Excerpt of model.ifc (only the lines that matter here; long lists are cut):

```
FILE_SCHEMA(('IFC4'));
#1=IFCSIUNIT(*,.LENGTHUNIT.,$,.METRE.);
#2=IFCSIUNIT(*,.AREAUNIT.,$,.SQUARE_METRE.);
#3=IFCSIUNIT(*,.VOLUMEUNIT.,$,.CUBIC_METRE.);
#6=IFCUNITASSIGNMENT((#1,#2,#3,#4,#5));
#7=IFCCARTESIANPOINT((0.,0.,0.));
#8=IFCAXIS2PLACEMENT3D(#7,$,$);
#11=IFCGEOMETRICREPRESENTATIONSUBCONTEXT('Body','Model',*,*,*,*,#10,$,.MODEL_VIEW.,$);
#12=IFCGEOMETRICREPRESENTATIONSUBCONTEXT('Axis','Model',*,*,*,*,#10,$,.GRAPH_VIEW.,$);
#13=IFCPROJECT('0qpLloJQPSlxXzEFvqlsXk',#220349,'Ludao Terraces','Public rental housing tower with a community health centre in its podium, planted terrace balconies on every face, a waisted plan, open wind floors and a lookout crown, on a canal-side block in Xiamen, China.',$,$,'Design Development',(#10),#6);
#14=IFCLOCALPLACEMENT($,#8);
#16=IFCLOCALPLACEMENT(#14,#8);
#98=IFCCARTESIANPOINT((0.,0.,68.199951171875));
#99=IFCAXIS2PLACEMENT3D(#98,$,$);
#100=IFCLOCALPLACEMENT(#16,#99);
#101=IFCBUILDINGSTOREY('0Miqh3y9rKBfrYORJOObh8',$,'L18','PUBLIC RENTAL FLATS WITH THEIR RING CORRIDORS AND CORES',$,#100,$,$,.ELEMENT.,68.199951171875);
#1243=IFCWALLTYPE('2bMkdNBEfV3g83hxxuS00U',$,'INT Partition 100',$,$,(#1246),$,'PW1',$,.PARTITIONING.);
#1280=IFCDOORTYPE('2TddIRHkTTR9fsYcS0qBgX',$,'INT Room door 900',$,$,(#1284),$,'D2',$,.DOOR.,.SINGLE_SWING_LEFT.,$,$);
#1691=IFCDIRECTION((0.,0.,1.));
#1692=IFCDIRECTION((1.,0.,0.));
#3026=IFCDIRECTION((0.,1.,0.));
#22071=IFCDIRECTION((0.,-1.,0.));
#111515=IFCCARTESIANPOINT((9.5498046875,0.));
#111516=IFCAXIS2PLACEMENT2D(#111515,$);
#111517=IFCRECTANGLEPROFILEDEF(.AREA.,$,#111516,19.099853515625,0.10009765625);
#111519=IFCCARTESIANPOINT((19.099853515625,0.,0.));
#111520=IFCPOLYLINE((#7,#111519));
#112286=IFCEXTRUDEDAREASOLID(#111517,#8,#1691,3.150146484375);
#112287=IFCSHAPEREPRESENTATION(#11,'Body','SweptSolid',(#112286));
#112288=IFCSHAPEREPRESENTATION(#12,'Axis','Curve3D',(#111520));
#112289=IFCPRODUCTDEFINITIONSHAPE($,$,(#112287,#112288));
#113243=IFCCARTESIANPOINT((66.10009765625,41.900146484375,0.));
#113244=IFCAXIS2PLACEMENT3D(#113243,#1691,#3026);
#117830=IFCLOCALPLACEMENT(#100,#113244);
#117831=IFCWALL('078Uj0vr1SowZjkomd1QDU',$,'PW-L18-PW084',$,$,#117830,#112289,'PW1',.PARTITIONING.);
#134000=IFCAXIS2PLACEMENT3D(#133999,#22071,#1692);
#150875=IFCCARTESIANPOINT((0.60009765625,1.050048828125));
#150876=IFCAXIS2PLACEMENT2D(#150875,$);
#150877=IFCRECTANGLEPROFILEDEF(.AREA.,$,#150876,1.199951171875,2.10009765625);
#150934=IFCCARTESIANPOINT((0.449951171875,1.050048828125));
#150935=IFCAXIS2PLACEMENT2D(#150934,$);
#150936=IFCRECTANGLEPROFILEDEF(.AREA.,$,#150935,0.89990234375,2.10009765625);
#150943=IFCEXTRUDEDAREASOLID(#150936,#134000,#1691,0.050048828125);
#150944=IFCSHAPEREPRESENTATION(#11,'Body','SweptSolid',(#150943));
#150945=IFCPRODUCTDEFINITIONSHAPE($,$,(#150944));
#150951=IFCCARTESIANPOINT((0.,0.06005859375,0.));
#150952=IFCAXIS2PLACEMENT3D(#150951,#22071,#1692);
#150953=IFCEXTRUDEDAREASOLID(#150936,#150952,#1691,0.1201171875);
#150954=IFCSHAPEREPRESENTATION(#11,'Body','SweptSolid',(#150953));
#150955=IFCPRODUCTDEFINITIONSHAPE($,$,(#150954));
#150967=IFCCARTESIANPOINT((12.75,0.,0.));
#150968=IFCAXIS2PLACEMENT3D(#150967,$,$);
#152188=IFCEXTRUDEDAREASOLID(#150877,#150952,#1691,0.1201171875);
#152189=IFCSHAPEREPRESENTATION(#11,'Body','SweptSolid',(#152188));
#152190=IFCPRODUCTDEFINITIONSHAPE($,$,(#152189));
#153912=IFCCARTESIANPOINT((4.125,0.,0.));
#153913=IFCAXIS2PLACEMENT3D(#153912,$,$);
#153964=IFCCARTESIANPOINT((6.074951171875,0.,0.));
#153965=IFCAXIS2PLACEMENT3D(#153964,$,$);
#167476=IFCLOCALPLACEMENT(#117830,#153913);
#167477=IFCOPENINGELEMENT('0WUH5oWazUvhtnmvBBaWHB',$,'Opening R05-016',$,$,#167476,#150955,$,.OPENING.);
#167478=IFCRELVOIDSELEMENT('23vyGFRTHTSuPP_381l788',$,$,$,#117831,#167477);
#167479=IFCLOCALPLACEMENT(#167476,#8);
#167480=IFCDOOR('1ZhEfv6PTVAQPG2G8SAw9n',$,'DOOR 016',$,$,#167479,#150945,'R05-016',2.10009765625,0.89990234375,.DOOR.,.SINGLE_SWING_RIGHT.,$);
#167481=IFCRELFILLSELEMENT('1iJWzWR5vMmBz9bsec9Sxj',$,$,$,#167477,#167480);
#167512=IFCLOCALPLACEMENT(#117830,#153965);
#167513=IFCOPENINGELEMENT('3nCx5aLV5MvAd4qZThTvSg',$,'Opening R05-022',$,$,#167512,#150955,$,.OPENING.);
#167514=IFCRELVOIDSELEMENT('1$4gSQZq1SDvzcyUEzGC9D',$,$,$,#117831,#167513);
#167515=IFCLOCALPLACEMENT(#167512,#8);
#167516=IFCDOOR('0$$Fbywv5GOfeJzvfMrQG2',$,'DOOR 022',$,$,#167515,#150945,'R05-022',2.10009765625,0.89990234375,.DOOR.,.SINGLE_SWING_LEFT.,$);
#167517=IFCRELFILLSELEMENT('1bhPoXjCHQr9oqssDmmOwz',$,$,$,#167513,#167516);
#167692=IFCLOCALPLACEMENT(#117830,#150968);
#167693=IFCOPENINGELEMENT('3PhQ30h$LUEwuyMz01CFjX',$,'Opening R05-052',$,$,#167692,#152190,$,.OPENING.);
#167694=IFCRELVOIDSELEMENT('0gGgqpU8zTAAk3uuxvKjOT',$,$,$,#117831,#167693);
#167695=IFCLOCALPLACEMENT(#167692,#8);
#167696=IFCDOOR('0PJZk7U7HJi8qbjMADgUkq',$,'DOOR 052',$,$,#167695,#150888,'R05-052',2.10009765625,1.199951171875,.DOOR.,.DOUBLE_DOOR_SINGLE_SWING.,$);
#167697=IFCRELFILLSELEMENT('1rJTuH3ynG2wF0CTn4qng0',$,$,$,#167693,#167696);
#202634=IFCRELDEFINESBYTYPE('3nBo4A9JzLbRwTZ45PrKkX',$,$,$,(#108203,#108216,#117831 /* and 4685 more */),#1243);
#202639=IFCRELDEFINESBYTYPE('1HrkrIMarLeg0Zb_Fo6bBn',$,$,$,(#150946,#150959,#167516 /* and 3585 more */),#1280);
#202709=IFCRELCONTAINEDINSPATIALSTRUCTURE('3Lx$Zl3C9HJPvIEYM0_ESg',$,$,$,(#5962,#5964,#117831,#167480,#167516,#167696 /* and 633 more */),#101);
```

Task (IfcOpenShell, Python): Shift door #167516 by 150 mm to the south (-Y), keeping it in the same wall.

```python
import ifcopenshell
import ifcopenshell.api.geometry
import ifcopenshell.util.placement
import ifcopenshell.util.unit

model = ifcopenshell.open("model.ifc")
unit_scale = ifcopenshell.util.unit.calculate_unit_scale(model)

door = model.by_guid("0$$Fbywv5GOfeJzvfMrQG2")
opening = door.FillsVoids[0].RelatingOpeningElement
wall = opening.VoidsElements[0].RelatingBuildingElement

wall_matrix = ifcopenshell.util.placement.get_local_placement(wall.ObjectPlacement)
shift = wall_matrix[:3, 0] * -0.15 / unit_scale
before = ifcopenshell.util.placement.get_local_placement(door.ObjectPlacement)[:3, 3].copy()

# The door is placed relative to its opening, so it follows when the opening moves.
matrix = ifcopenshell.util.placement.get_local_placement(opening.ObjectPlacement)
matrix[:3, 3] += shift
ifcopenshell.api.geometry.edit_object_placement(
    model, product=opening, matrix=matrix, is_si=False, should_transform_children=True
)

after = ifcopenshell.util.placement.get_local_placement(door.ObjectPlacement)[:3, 3]
print("door moved by", (after - before).round(3) + 0.0)

model.write("model-out.ifc")
```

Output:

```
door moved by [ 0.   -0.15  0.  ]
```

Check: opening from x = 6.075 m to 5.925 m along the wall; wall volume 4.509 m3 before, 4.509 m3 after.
